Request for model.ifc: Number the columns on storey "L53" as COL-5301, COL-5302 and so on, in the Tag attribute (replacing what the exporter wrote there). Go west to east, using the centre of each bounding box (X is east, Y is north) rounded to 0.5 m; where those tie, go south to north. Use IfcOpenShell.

First a look at what the model holds.

```python
import ifcopenshell
import ifcopenshell.util.element
import ifcopenshell.util.placement

model = ifcopenshell.open("model.ifc")
print(model.schema)
storey = next(s for s in model.by_type("IfcBuildingStorey") if s.Name == "L53")
columns = [e for e in ifcopenshell.util.element.get_decomposition(storey) if e.is_a("IfcColumn")]
for e in sorted(columns, key=lambda e: e.id()):
    origin = ifcopenshell.util.placement.get_local_placement(e.ObjectPlacement)[:3, 3]
    print(e.id(), e.Tag, e.Name, origin.round(2) + 0.0, sep=" | ")
```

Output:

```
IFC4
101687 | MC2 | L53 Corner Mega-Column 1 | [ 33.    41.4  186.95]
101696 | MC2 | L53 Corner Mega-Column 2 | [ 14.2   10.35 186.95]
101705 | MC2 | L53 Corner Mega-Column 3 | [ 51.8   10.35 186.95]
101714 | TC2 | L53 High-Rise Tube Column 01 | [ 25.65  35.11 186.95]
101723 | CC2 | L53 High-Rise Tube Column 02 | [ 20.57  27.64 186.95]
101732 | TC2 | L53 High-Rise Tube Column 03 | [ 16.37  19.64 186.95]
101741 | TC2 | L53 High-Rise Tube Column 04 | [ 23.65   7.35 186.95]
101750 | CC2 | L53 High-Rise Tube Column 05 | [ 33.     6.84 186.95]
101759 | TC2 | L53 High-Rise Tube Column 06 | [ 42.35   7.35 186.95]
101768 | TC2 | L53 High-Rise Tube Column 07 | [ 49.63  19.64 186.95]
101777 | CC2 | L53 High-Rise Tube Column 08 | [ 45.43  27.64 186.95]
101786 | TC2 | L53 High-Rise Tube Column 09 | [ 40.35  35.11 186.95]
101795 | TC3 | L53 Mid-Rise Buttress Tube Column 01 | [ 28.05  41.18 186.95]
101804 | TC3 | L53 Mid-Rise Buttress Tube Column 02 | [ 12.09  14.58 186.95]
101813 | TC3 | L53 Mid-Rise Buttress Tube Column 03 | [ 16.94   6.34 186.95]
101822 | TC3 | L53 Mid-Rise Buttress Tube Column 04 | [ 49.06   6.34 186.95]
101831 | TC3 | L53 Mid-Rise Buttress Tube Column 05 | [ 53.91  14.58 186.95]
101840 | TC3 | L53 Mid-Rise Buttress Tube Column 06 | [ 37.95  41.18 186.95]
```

```python
import ifcopenshell
import ifcopenshell.geom
import ifcopenshell.util.element
import ifcopenshell.util.shape

model = ifcopenshell.open("model.ifc")
settings = ifcopenshell.geom.settings()
settings.set("use-world-coords", True)


def centre(element):
    shape = ifcopenshell.geom.create_shape(settings, element)
    return ifcopenshell.util.shape.get_bbox_centroid(shape.geometry)


storey = next(s for s in model.by_type("IfcBuildingStorey") if s.Name == "L53")
columns = [e for e in ifcopenshell.util.element.get_decomposition(storey) if e.is_a("IfcColumn")]

# Insertion points can sit at a corner or the storey origin, so sort by the geometry (in metres).
centres = {e: centre(e) for e in columns}
columns.sort(key=lambda e: (round(centres[e][0] / 0.5), centres[e][1]))

for i, e in enumerate(columns, start=1):
    number = f"COL-53{i:02d}"
    e.Tag = number
    print(e.id(), number)

model.write("model-out.ifc")
```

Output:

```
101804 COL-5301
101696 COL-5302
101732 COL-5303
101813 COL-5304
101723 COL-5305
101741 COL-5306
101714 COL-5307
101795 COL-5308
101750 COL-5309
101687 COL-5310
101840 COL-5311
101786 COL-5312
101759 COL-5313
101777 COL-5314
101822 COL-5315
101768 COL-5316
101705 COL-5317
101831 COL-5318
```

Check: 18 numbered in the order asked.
